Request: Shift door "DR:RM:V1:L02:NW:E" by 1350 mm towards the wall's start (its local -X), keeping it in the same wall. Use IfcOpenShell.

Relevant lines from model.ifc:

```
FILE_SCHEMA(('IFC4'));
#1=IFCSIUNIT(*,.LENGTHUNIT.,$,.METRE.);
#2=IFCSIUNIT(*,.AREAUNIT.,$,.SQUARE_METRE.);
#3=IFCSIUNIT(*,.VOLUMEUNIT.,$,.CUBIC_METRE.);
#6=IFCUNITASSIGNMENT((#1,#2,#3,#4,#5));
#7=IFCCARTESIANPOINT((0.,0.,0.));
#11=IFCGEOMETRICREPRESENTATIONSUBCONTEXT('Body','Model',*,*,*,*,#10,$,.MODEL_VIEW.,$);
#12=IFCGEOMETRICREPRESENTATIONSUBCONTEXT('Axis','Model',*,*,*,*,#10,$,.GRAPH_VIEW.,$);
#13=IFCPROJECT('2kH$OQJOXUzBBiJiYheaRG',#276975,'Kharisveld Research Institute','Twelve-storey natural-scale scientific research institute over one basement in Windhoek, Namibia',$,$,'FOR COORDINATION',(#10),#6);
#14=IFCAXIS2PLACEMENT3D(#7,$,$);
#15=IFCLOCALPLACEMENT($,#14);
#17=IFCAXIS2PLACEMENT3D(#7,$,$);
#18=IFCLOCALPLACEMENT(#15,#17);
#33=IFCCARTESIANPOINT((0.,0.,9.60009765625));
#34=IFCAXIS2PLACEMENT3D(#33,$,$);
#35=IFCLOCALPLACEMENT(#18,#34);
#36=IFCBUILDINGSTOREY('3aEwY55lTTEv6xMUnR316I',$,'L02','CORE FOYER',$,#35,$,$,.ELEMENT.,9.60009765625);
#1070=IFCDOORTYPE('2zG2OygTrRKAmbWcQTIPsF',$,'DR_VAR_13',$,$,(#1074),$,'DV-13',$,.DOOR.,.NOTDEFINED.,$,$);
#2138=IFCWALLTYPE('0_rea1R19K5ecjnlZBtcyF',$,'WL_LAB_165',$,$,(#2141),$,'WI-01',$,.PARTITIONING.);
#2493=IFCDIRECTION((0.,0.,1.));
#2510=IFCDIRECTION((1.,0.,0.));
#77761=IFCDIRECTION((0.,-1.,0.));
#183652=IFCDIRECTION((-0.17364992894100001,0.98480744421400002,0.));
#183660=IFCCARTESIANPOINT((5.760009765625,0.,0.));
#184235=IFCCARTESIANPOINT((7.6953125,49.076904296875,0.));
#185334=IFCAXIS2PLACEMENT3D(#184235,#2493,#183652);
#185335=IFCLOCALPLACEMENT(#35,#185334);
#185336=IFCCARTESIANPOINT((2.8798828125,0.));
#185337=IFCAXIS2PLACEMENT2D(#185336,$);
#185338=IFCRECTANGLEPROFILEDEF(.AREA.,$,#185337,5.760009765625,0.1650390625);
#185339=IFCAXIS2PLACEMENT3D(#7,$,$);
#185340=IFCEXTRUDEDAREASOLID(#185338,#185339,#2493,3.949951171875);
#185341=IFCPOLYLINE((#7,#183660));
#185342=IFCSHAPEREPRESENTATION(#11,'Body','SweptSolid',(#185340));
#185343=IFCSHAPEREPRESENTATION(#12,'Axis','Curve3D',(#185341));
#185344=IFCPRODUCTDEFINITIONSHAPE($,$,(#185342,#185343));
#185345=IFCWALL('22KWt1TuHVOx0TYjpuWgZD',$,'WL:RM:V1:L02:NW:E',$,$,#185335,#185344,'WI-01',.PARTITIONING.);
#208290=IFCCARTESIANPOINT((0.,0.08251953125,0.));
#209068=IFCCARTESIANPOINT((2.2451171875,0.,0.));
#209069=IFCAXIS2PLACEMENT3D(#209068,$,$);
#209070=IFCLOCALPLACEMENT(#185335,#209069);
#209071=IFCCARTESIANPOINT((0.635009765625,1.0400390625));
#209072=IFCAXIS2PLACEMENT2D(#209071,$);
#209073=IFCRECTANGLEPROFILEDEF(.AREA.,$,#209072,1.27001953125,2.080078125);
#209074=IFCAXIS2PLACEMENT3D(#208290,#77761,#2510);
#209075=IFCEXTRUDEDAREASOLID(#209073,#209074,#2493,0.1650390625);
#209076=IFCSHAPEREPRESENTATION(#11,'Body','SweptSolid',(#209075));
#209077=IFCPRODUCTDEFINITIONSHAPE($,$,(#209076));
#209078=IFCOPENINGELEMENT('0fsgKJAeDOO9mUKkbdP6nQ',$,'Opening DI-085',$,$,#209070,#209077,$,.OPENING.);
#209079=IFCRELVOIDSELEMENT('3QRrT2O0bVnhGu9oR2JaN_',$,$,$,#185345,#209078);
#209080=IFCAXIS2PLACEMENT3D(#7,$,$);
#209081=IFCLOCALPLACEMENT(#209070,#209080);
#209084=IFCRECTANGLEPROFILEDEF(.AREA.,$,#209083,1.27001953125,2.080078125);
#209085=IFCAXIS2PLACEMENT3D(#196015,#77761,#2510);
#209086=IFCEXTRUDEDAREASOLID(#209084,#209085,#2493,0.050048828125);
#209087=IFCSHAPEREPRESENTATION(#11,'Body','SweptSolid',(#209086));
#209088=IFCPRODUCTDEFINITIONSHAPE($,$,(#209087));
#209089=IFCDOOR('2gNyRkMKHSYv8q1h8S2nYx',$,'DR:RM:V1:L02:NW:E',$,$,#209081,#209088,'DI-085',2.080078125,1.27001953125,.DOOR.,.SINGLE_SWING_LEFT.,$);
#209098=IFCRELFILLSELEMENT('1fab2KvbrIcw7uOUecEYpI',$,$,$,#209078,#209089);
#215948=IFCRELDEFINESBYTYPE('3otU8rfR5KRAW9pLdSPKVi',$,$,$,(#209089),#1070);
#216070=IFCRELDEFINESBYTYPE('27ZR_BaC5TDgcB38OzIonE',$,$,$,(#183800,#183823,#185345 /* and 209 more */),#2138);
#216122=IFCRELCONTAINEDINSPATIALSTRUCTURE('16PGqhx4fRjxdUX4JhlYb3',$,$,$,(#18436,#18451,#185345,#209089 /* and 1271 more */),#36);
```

```python
import ifcopenshell
import ifcopenshell.api.geometry
import ifcopenshell.util.placement
import ifcopenshell.util.unit

model = ifcopenshell.open("model.ifc")
unit_scale = ifcopenshell.util.unit.calculate_unit_scale(model)

door = model.by_guid("2gNyRkMKHSYv8q1h8S2nYx")
opening = door.FillsVoids[0].RelatingOpeningElement
wall = opening.VoidsElements[0].RelatingBuildingElement

wall_matrix = ifcopenshell.util.placement.get_local_placement(wall.ObjectPlacement)
shift = wall_matrix[:3, 0] * -1.35 / unit_scale
before = ifcopenshell.util.placement.get_local_placement(door.ObjectPlacement)[:3, 3].copy()

# The door is placed relative to its opening, so it follows when the opening moves.
matrix = ifcopenshell.util.placement.get_local_placement(opening.ObjectPlacement)
matrix[:3, 3] += shift
ifcopenshell.api.geometry.edit_object_placement(
    model, product=opening, matrix=matrix, is_si=False, should_transform_children=True
)

after = ifcopenshell.util.placement.get_local_placement(door.ObjectPlacement)[:3, 3]
print("door moved by", (after - before).round(3) + 0.0)

model.write("model_updated.ifc")
```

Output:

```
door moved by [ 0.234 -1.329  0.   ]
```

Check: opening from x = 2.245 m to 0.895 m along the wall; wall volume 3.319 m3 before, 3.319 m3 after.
